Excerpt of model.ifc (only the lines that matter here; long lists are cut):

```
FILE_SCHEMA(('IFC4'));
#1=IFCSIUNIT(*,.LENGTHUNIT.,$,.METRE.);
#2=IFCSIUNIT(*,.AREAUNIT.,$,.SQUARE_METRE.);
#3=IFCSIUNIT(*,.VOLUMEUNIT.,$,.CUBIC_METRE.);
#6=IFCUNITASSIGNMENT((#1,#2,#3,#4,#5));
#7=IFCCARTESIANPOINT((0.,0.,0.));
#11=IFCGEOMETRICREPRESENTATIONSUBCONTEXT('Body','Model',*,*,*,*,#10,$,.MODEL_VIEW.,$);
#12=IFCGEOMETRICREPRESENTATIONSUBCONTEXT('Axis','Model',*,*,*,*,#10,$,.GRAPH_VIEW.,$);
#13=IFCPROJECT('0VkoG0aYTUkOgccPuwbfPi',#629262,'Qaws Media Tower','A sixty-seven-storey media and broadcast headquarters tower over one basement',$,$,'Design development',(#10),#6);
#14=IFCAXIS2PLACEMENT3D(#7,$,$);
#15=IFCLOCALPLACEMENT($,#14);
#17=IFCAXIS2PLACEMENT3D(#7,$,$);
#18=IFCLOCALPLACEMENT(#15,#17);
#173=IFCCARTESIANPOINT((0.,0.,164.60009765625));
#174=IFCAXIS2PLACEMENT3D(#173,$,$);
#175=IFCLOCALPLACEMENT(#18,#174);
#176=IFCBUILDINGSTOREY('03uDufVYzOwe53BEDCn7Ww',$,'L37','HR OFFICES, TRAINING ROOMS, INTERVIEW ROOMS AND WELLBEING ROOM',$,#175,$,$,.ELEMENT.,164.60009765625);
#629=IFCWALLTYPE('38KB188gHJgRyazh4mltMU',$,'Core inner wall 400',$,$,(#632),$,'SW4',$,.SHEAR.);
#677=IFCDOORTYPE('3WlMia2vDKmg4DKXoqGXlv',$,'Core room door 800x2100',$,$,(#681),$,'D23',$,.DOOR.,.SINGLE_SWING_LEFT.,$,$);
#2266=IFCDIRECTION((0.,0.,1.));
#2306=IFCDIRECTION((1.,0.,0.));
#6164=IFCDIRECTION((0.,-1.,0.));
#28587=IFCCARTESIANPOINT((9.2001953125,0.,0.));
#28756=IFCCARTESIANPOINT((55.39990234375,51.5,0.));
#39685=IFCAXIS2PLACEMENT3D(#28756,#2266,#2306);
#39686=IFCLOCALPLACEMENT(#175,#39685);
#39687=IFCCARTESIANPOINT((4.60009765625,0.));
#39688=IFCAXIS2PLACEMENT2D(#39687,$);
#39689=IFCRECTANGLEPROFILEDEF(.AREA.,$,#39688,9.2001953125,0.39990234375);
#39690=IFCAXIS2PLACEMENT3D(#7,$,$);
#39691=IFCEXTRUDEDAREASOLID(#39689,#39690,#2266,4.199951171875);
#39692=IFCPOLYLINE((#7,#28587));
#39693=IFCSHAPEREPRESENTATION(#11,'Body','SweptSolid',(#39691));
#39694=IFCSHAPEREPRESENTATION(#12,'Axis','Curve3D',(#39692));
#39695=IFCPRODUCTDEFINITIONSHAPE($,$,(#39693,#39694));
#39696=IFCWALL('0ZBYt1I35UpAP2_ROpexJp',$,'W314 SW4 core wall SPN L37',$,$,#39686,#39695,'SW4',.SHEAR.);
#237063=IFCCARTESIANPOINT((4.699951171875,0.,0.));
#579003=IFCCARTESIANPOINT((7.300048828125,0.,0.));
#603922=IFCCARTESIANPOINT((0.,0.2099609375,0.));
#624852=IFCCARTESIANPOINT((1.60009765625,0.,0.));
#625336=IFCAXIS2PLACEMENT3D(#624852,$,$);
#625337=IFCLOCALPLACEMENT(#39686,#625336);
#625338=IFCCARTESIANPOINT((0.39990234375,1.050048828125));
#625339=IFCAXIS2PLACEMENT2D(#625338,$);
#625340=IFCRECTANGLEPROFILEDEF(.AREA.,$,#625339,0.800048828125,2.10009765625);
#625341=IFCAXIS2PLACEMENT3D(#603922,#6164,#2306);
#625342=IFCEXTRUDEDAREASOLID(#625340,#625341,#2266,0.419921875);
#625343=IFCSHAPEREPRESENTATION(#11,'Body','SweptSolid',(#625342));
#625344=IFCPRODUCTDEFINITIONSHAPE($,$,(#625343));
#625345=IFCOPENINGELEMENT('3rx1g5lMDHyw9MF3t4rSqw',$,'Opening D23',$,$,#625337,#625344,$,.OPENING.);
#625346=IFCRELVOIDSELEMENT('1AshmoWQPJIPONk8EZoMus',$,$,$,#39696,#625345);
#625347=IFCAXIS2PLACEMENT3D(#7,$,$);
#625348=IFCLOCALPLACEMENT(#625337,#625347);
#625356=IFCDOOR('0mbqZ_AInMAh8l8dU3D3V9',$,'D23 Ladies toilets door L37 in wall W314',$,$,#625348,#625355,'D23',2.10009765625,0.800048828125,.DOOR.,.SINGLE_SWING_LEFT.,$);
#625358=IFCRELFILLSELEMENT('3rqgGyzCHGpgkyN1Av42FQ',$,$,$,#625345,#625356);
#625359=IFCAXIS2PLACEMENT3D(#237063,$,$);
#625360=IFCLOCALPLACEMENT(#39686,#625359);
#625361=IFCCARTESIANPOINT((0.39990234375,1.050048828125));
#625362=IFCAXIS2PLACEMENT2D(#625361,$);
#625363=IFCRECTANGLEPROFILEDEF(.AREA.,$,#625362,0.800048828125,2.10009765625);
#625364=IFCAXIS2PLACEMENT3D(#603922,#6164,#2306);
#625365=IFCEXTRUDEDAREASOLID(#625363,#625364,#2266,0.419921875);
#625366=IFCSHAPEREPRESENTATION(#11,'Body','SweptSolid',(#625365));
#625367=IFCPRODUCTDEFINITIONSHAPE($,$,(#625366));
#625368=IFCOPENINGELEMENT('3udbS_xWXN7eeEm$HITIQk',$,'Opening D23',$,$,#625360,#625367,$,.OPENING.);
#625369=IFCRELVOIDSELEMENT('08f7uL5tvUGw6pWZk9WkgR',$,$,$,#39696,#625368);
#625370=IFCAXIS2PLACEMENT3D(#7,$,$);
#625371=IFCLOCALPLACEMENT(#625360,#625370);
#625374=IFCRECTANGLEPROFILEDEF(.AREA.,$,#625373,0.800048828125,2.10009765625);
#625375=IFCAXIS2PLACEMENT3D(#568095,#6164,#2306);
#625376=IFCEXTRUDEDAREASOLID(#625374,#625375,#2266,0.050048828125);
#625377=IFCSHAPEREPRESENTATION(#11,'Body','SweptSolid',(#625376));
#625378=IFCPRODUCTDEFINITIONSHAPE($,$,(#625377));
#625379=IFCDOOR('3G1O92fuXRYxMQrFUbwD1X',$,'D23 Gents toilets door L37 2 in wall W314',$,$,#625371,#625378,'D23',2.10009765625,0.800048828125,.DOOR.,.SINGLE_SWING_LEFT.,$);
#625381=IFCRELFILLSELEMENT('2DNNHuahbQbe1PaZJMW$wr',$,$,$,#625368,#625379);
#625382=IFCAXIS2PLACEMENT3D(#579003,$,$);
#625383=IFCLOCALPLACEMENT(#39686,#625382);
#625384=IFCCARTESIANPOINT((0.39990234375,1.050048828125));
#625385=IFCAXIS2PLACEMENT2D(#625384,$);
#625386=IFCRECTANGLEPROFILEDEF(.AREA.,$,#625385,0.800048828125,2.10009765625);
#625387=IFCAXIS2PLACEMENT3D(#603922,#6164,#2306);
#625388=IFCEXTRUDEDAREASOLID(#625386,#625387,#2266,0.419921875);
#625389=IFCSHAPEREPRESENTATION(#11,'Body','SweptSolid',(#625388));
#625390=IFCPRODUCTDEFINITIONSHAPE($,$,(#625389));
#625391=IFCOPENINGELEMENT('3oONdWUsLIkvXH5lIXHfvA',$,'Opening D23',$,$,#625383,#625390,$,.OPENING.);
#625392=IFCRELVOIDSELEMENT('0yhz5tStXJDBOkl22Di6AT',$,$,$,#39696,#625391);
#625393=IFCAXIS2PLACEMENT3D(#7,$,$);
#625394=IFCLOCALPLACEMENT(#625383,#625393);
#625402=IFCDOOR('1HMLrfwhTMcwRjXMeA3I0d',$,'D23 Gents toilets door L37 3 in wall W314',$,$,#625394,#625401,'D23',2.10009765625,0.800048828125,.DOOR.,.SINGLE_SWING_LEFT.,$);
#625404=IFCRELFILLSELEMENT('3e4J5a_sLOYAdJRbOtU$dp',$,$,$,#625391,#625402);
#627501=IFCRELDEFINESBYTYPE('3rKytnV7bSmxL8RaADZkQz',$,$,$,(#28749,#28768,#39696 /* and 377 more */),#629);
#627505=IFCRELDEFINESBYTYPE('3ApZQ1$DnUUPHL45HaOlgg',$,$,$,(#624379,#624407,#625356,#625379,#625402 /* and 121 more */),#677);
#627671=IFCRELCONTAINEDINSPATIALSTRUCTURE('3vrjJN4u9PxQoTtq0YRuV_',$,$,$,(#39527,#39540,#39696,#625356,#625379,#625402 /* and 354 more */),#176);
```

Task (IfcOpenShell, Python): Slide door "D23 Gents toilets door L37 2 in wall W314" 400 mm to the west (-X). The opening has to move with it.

```python
import ifcopenshell
import ifcopenshell.api.geometry
import ifcopenshell.util.placement
import ifcopenshell.util.unit

model = ifcopenshell.open("model.ifc")
unit_scale = ifcopenshell.util.unit.calculate_unit_scale(model)

door = model.by_guid("3G1O92fuXRYxMQrFUbwD1X")
opening = door.FillsVoids[0].RelatingOpeningElement
wall = opening.VoidsElements[0].RelatingBuildingElement

wall_matrix = ifcopenshell.util.placement.get_local_placement(wall.ObjectPlacement)
shift = wall_matrix[:3, 0] * -0.4 / unit_scale
before = ifcopenshell.util.placement.get_local_placement(door.ObjectPlacement)[:3, 3].copy()

# The door is placed relative to its opening, so it follows when the opening moves.
matrix = ifcopenshell.util.placement.get_local_placement(opening.ObjectPlacement)
matrix[:3, 3] += shift
ifcopenshell.api.geometry.edit_object_placement(
    model, product=opening, matrix=matrix, is_si=False, should_transform_children=True
)

after = ifcopenshell.util.placement.get_local_placement(door.ObjectPlacement)[:3, 3]
print("door moved by", (after - before).round(3) + 0.0)

model.write("model_v2.ifc")
```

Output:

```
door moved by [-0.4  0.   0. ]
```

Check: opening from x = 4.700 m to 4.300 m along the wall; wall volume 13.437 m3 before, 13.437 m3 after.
